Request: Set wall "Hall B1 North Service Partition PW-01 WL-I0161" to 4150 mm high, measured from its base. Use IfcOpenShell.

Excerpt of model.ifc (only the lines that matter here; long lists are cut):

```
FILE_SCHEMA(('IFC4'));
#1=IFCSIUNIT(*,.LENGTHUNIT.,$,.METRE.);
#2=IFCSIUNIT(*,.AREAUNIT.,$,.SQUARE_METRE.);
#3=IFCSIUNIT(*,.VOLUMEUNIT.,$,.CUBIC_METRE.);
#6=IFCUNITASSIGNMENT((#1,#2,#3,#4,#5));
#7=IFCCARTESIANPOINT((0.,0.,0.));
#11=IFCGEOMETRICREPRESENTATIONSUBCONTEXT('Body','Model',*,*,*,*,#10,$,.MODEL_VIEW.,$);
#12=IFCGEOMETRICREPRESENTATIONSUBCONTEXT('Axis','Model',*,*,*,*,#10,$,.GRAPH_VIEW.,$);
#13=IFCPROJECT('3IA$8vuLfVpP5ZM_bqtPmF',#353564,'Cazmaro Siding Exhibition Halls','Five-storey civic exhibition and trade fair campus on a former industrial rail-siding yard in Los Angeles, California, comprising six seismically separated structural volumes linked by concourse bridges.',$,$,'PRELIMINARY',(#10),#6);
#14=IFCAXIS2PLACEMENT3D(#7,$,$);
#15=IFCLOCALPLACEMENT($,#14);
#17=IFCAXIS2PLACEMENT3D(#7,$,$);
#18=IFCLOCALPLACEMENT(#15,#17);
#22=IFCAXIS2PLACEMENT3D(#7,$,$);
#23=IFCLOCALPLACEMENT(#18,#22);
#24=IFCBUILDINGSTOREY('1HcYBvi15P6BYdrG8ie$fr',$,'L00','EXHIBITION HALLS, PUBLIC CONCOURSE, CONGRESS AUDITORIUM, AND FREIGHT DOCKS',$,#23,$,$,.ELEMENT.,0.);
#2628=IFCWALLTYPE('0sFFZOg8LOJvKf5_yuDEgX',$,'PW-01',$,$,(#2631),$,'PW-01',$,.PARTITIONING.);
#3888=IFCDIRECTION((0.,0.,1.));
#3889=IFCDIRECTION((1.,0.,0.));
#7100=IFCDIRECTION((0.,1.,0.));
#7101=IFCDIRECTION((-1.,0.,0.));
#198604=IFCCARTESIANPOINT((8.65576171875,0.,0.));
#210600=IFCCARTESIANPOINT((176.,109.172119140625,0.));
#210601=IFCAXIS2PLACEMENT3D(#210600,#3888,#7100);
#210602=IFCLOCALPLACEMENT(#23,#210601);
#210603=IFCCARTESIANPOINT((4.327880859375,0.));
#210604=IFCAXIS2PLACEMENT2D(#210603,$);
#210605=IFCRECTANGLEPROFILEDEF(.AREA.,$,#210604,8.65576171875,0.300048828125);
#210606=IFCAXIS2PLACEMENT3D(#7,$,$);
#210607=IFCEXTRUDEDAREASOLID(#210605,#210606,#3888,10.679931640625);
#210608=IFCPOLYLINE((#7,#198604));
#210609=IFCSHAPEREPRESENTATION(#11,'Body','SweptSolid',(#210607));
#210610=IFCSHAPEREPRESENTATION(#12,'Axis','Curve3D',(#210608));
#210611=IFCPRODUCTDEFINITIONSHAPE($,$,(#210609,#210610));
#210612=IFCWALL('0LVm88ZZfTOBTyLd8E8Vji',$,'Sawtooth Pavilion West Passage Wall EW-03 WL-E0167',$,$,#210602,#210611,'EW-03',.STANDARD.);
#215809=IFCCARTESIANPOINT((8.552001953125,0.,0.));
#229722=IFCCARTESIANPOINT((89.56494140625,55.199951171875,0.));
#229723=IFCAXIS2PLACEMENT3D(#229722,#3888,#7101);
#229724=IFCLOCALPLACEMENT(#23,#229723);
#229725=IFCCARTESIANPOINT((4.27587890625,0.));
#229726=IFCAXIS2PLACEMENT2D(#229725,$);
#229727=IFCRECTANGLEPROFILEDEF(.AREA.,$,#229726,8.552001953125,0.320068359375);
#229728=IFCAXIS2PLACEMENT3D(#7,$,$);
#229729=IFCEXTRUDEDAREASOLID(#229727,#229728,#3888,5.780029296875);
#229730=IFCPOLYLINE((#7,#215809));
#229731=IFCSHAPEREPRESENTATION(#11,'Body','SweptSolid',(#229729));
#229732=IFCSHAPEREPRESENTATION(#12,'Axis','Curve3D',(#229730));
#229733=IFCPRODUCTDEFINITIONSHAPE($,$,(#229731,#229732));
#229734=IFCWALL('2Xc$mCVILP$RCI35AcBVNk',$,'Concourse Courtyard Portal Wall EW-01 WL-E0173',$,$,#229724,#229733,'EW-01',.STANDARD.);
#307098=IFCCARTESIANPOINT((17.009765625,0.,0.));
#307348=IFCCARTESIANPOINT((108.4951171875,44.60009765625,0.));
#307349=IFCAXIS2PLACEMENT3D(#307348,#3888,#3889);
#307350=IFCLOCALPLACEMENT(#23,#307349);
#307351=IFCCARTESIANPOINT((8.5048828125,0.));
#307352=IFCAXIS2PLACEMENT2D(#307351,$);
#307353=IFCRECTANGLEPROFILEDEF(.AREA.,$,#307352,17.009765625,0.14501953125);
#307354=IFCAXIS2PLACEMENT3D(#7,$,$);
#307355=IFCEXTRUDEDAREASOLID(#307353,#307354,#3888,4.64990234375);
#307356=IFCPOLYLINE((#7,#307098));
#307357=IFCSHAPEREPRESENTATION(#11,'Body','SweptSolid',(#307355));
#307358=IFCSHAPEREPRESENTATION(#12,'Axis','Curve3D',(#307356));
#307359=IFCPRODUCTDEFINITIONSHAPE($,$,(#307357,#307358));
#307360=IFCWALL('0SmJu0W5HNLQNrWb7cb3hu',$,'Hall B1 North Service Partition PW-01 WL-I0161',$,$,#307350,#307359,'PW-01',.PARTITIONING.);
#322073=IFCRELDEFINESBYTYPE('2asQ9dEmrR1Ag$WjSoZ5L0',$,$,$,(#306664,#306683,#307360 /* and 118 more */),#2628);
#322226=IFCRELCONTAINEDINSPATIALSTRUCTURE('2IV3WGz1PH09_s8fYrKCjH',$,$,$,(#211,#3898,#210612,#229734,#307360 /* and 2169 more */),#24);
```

```python
import ifcopenshell
import ifcopenshell.geom
import ifcopenshell.util.representation
import ifcopenshell.util.shape
import ifcopenshell.util.unit

model = ifcopenshell.open("model.ifc")
unit_scale = ifcopenshell.util.unit.calculate_unit_scale(model)
settings = ifcopenshell.geom.settings()


def volume(element):
    """Net volume in cubic metres, openings subtracted."""
    shape = ifcopenshell.geom.create_shape(settings, element)
    return ifcopenshell.util.shape.get_volume(shape.geometry)


wall = model.by_id(307360)
before = volume(wall)

body = ifcopenshell.util.representation.get_representation(wall, "Model", "Body")
solid = body.Items[0]
old_height = solid.Depth
solid.Depth = 4.15 / unit_scale
after = volume(wall)

print(f"height {old_height:g} -> {solid.Depth:g}, volume {before:.3f} -> {after:.3f} m3")

model.write("model_v2.ifc")
```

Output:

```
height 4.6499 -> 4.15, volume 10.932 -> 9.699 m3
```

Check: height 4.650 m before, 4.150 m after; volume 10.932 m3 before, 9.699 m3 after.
